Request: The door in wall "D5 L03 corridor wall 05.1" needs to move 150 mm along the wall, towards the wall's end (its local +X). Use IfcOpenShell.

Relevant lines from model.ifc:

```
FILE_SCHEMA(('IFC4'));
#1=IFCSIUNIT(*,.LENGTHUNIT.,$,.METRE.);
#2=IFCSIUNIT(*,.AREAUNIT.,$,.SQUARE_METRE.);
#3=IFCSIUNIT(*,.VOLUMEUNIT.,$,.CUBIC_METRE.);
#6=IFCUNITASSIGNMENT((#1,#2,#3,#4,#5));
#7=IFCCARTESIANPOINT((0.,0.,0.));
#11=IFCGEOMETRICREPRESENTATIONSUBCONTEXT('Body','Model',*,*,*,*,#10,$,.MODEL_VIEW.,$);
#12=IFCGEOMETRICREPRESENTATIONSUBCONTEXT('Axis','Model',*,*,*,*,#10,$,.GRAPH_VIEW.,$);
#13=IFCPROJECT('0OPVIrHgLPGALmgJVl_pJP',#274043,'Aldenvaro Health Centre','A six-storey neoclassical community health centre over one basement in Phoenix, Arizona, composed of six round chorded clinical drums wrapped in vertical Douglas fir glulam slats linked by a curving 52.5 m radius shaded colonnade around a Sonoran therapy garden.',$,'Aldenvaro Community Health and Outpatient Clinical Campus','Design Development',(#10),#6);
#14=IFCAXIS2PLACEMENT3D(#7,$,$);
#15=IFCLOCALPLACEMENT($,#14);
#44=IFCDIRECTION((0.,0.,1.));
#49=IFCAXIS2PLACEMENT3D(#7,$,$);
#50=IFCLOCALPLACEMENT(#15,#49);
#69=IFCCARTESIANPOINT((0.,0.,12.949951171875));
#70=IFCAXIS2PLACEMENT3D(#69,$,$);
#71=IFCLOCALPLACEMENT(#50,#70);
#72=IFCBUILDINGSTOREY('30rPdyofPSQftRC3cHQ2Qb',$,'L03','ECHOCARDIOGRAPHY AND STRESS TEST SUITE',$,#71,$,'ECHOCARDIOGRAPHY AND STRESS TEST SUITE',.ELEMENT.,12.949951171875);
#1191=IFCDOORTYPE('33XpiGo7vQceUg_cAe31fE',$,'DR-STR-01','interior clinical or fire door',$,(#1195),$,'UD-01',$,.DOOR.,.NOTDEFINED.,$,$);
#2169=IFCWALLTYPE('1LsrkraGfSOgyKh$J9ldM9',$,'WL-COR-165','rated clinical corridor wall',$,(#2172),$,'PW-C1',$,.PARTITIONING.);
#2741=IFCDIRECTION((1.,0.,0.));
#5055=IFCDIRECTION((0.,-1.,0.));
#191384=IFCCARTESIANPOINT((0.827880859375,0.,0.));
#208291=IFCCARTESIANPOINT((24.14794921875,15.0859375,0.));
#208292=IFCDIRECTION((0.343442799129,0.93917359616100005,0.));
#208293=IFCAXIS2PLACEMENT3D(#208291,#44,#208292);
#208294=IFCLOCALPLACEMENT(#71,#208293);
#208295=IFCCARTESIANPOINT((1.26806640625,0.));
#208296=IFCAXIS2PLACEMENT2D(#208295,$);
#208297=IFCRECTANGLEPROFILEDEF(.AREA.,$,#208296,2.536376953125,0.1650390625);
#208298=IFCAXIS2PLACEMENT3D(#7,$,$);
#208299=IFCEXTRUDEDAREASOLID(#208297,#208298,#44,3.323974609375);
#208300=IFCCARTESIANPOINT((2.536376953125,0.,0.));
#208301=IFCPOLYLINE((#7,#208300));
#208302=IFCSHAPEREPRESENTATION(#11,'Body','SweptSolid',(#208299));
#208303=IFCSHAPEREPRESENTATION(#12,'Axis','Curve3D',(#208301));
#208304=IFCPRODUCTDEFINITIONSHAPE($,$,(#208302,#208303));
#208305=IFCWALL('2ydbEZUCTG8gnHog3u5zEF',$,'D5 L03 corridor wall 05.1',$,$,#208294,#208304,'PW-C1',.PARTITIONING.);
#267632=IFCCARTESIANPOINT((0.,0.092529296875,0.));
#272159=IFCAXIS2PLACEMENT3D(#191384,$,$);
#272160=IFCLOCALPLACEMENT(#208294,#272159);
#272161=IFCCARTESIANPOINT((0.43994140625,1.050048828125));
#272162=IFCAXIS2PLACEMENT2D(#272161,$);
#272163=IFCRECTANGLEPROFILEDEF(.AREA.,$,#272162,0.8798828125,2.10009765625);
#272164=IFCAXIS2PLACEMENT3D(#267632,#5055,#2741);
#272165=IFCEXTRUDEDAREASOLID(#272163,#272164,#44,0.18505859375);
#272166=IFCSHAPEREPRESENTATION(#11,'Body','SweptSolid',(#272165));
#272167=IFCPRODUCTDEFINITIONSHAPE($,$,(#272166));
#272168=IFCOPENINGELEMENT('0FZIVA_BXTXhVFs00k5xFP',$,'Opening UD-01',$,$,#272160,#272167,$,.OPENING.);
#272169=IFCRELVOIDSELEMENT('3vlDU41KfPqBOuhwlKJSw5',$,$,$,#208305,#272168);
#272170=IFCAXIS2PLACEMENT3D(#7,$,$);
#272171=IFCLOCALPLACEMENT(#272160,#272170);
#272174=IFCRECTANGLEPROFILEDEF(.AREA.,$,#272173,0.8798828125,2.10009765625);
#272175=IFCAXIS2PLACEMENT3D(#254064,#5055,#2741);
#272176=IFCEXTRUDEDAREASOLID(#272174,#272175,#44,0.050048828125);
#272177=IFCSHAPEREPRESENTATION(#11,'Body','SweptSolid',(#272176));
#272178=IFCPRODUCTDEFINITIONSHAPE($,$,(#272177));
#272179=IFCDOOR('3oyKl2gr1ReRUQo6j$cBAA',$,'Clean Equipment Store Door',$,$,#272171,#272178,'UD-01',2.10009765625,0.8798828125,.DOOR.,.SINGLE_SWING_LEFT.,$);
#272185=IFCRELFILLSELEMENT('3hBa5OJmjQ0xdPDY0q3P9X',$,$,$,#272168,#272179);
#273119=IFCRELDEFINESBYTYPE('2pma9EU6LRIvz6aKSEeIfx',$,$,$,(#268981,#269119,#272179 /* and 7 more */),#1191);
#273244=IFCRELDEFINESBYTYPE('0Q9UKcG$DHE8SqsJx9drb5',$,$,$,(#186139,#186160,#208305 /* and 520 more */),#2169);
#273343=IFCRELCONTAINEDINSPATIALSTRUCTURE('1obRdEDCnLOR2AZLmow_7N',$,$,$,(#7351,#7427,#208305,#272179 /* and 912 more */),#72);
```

```python
import ifcopenshell
import ifcopenshell.api.geometry
import ifcopenshell.util.placement

model = ifcopenshell.open("model.ifc")

door = model.by_guid("3oyKl2gr1ReRUQo6j$cBAA")
opening = door.FillsVoids[0].RelatingOpeningElement
wall = opening.VoidsElements[0].RelatingBuildingElement

wall_matrix = ifcopenshell.util.placement.get_local_placement(wall.ObjectPlacement)
shift = wall_matrix[:3, 0] * 0.15
before = ifcopenshell.util.placement.get_local_placement(door.ObjectPlacement)[:3, 3].copy()

# The door is placed relative to its opening, so it follows when the opening moves.
matrix = ifcopenshell.util.placement.get_local_placement(opening.ObjectPlacement)
matrix[:3, 3] += shift
ifcopenshell.api.geometry.edit_object_placement(
    model, product=opening, matrix=matrix, is_si=False, should_transform_children=True
)

after = ifcopenshell.util.placement.get_local_placement(door.ObjectPlacement)[:3, 3]
print("door moved by", (after - before).round(3) + 0.0)

model.write("model_edited.ifc")
```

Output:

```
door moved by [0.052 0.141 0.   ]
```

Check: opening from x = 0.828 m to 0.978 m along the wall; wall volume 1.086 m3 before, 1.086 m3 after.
